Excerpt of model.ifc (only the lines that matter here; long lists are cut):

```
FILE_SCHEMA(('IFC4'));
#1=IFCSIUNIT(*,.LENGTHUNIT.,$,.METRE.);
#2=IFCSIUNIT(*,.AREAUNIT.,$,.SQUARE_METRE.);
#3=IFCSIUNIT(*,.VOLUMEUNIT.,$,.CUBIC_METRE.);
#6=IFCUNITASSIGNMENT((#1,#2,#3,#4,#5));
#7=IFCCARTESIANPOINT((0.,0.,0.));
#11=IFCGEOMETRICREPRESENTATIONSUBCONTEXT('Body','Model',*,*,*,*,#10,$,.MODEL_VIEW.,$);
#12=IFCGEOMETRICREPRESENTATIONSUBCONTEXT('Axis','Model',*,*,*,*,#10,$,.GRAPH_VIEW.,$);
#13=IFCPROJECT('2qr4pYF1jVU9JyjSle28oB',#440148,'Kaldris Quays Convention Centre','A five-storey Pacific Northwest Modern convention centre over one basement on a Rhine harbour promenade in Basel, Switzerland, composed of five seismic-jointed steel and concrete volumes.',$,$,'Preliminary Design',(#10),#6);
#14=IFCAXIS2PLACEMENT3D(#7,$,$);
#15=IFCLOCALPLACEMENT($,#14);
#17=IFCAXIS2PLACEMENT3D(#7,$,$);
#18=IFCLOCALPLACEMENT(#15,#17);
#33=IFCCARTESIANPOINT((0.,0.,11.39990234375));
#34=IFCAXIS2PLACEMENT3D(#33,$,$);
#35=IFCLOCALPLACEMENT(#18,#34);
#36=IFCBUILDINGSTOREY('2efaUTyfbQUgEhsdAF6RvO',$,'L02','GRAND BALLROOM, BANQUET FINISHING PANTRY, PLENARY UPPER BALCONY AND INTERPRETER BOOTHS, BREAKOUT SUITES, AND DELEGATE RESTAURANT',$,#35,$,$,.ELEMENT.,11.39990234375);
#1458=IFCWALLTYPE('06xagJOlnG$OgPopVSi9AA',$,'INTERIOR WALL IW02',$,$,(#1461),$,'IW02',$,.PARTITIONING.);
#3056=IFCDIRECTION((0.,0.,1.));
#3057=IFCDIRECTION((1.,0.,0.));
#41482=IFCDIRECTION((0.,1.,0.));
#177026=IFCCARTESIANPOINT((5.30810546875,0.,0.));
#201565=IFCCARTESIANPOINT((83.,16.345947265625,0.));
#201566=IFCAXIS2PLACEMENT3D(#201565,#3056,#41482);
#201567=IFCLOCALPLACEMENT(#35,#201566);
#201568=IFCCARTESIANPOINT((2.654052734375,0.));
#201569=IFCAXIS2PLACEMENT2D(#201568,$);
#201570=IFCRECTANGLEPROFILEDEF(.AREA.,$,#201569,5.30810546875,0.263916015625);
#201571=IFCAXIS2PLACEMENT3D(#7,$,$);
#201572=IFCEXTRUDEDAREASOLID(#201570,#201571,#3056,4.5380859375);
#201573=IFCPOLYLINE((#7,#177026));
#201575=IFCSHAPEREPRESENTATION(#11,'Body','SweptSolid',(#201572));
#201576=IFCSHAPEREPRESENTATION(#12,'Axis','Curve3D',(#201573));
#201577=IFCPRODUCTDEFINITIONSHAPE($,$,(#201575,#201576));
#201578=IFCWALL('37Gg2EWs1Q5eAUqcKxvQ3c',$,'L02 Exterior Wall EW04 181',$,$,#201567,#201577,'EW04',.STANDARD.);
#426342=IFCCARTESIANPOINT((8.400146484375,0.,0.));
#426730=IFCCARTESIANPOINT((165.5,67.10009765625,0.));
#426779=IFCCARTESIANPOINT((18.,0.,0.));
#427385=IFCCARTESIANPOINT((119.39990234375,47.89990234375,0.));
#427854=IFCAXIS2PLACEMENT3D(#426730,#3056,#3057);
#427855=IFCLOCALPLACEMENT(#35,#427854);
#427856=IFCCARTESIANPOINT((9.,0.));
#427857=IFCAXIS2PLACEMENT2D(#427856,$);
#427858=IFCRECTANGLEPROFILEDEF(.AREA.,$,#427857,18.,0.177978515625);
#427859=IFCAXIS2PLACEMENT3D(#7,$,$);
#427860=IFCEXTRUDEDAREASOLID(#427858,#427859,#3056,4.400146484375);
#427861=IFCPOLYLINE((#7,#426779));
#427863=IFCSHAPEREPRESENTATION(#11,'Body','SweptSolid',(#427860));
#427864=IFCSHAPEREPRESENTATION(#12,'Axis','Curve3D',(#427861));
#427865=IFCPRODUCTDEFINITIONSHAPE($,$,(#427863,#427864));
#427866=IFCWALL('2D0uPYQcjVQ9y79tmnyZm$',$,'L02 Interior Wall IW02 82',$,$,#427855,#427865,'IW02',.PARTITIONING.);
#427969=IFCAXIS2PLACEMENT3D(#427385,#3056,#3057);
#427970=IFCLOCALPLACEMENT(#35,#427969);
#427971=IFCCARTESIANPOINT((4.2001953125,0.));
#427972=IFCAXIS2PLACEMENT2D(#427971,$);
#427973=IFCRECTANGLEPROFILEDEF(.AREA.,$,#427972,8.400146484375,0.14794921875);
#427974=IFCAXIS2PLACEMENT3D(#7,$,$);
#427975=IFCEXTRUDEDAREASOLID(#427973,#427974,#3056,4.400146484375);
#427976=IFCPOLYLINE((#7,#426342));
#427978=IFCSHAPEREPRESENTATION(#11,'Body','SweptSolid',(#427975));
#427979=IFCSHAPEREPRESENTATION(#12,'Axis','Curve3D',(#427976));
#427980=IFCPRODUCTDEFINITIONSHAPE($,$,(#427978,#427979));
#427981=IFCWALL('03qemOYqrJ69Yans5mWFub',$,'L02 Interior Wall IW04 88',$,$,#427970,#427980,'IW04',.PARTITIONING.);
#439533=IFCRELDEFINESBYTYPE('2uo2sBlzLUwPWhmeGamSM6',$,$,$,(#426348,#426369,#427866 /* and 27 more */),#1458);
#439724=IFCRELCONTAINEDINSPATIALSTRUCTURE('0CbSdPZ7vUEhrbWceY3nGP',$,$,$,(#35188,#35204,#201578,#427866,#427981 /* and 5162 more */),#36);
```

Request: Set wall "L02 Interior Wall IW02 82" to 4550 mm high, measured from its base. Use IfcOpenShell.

```python
import ifcopenshell
import ifcopenshell.geom
import ifcopenshell.util.representation
import ifcopenshell.util.shape
import ifcopenshell.util.unit

model = ifcopenshell.open("model.ifc")
unit_scale = ifcopenshell.util.unit.calculate_unit_scale(model)
settings = ifcopenshell.geom.settings()


def volume(element):
    """Net volume in cubic metres, openings subtracted."""
    shape = ifcopenshell.geom.create_shape(settings, element)
    return ifcopenshell.util.shape.get_volume(shape.geometry)


wall = model.by_id(427866)
before = volume(wall)

body = ifcopenshell.util.representation.get_representation(wall, "Model", "Body")
solid = body.Items[0]
old_height = solid.Depth
solid.Depth = 4.55 / unit_scale
after = volume(wall)

print(f"height {old_height:g} -> {solid.Depth:g}, volume {before:.3f} -> {after:.3f} m3")

model.write("model_v2.ifc")
```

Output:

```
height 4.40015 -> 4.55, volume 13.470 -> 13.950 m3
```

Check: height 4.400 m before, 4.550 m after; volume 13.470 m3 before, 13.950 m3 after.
